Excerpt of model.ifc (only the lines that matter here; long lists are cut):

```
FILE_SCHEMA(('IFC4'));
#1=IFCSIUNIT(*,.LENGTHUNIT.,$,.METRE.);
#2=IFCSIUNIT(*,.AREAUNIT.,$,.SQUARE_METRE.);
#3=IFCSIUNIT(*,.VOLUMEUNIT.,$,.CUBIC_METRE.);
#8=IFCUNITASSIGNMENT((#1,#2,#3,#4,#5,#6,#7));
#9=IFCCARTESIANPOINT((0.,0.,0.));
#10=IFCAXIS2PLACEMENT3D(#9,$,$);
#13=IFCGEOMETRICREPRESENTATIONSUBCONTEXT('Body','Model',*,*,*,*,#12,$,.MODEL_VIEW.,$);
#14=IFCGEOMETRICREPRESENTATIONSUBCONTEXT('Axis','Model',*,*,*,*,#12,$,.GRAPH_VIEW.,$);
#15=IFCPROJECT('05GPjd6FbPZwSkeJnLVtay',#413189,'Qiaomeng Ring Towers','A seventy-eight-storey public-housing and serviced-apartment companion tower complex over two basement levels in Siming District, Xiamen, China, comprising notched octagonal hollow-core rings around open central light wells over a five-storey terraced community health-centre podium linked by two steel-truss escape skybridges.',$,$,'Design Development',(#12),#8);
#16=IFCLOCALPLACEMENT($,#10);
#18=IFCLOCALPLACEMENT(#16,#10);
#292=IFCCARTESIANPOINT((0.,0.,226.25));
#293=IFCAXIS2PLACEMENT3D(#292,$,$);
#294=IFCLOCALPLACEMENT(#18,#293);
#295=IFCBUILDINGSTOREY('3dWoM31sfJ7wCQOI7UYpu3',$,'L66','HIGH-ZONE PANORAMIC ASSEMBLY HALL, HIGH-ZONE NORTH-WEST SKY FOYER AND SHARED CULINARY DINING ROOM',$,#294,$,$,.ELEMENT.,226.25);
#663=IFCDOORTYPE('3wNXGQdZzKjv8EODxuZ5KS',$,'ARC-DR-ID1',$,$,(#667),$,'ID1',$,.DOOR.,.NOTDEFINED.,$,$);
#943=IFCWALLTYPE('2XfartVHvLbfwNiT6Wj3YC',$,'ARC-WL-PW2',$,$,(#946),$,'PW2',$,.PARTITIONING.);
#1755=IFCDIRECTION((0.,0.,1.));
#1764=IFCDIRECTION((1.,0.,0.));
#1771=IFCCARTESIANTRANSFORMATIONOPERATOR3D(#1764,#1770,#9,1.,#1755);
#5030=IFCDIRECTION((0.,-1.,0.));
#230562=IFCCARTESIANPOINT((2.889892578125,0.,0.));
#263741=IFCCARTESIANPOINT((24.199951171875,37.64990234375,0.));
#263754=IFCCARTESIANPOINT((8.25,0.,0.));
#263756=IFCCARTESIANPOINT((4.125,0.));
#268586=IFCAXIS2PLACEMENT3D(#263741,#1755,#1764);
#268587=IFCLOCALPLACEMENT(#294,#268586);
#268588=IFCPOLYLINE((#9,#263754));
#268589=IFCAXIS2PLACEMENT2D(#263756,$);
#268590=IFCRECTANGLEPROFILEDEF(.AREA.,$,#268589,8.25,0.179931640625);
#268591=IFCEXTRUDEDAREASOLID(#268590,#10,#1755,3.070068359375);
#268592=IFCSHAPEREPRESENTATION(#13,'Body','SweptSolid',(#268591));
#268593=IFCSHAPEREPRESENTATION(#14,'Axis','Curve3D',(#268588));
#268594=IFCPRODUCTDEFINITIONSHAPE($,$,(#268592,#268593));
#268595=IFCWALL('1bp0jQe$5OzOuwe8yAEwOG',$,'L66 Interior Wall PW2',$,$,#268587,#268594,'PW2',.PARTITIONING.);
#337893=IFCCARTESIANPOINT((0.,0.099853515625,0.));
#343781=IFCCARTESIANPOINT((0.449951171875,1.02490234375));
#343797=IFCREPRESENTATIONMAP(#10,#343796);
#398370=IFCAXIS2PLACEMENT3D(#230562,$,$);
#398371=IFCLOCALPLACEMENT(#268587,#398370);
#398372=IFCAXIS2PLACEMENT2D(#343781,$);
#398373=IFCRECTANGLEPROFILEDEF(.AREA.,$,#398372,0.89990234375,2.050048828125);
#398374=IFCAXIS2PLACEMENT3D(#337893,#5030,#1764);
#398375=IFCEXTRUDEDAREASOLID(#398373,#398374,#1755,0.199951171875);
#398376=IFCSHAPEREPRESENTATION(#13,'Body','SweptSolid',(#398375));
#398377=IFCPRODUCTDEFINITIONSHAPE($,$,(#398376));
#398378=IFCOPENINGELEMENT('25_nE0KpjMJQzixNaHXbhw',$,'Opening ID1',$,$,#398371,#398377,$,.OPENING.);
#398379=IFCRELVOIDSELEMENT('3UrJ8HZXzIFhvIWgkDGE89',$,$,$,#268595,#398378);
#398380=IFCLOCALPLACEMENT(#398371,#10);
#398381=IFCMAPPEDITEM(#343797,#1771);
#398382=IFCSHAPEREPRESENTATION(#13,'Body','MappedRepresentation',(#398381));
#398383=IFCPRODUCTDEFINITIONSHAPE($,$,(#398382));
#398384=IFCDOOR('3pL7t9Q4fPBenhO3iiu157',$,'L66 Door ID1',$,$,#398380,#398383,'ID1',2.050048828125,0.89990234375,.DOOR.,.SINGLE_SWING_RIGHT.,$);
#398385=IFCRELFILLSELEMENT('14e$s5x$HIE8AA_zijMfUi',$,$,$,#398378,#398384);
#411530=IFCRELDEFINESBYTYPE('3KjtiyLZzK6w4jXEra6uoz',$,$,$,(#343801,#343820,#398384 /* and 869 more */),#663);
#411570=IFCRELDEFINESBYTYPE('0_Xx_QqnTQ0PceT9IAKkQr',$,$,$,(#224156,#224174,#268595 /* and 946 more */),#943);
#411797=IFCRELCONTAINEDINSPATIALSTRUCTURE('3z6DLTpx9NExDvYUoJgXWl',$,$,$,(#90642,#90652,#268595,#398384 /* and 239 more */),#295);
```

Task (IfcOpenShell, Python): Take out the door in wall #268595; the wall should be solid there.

```python
import ifcopenshell
import ifcopenshell.api.feature
import ifcopenshell.api.root
import ifcopenshell.geom
import ifcopenshell.util.shape

model = ifcopenshell.open("model.ifc")
settings = ifcopenshell.geom.settings()


def volume(element):
    """Net volume in cubic metres, openings subtracted."""
    shape = ifcopenshell.geom.create_shape(settings, element)
    return ifcopenshell.util.shape.get_volume(shape.geometry)


door = model.by_guid("3pL7t9Q4fPBenhO3iiu157")
opening = door.FillsVoids[0].RelatingOpeningElement
wall = opening.VoidsElements[0].RelatingBuildingElement
before = volume(wall)

ifcopenshell.api.root.remove_product(model, product=door)
ifcopenshell.api.feature.remove_feature(model, feature=opening)

after = volume(wall)

print(f"wall volume {before:.3f} -> {after:.3f} m3")

model.write("model_rev.ifc")
```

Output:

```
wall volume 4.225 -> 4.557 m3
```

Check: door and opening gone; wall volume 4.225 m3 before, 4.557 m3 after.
